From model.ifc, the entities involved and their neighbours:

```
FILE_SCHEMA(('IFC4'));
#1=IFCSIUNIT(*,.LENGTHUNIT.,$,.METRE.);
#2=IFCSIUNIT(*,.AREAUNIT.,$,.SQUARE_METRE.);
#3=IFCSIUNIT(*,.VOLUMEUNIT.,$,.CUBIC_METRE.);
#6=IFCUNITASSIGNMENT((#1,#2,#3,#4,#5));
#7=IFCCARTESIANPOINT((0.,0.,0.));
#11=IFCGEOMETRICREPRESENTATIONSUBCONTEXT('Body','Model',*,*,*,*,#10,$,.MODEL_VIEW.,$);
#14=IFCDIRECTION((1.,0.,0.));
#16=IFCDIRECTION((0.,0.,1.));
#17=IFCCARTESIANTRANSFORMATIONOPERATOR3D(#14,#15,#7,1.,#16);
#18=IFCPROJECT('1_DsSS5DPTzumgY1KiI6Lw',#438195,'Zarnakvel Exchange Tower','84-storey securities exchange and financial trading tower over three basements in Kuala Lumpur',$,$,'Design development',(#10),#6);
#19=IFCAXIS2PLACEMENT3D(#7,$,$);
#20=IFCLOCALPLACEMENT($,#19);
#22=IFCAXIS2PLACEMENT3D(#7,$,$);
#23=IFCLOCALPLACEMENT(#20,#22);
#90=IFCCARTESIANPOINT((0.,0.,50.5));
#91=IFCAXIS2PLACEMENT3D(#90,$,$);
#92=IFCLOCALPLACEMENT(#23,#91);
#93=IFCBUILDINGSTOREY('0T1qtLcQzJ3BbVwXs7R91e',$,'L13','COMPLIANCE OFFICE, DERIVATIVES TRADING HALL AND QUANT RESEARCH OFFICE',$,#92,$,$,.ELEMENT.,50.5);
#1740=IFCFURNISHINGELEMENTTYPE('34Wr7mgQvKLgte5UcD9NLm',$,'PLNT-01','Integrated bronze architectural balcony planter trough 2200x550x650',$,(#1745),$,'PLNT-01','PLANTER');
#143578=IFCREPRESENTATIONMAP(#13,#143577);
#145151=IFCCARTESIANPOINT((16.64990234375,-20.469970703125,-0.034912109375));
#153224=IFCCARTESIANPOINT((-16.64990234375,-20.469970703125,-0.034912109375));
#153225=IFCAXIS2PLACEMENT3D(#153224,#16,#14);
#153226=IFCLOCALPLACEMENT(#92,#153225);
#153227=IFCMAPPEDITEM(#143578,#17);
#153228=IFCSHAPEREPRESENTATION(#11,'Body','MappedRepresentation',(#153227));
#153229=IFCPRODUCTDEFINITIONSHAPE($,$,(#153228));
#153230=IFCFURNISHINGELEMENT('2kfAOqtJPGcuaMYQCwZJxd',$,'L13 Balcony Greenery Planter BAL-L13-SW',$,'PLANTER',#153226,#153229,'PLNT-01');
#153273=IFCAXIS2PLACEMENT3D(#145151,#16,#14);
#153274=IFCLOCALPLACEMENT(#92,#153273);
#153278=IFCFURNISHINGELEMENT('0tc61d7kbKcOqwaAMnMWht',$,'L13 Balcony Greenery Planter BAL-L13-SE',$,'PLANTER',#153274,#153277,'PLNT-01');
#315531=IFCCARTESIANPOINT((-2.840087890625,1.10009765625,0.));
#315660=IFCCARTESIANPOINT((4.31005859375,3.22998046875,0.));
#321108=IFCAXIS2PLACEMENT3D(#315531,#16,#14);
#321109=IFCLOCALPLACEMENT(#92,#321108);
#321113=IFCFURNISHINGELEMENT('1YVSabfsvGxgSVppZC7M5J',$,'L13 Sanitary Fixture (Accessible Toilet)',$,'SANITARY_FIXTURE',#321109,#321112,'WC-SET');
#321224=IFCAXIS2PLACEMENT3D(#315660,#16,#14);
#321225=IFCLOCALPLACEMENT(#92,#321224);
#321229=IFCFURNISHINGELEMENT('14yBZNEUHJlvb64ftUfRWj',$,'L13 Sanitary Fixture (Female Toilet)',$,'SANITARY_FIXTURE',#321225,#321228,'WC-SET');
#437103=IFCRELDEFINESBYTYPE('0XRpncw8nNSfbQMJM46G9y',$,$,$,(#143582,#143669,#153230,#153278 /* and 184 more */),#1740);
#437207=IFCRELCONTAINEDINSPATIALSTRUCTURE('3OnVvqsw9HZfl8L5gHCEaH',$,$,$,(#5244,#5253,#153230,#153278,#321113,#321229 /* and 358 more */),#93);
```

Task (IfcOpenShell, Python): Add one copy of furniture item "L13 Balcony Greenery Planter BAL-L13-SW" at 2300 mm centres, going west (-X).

```python
import numpy as np
import ifcopenshell
import ifcopenshell.api.geometry
import ifcopenshell.api.root
import ifcopenshell.util.element
import ifcopenshell.util.placement
import ifcopenshell.util.unit

model = ifcopenshell.open("model.ifc")
unit_scale = ifcopenshell.util.unit.calculate_unit_scale(model)

source = model.by_guid("2kfAOqtJPGcuaMYQCwZJxd")
base = ifcopenshell.util.placement.get_local_placement(source.ObjectPlacement)
step = np.array([-1.0, 0.0, 0.0]) * 2.3 / unit_scale

for i in range(1, 2):
    copy = ifcopenshell.api.root.copy_class(model, product=source)
    copy.Representation = ifcopenshell.util.element.copy_deep(
        model, source.Representation, exclude=["IfcGeometricRepresentationContext", "IfcRepresentationMap"]
    )
    copy.Tag = None
    matrix = base.copy()
    matrix[:3, 3] += i * step
    print("added at", matrix[:3, 3].round(3) + 0.0)
    ifcopenshell.api.geometry.edit_object_placement(model, product=copy, matrix=matrix, is_si=False)

model.write("model_updated.ifc")
```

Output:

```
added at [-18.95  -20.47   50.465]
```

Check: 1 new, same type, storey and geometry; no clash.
